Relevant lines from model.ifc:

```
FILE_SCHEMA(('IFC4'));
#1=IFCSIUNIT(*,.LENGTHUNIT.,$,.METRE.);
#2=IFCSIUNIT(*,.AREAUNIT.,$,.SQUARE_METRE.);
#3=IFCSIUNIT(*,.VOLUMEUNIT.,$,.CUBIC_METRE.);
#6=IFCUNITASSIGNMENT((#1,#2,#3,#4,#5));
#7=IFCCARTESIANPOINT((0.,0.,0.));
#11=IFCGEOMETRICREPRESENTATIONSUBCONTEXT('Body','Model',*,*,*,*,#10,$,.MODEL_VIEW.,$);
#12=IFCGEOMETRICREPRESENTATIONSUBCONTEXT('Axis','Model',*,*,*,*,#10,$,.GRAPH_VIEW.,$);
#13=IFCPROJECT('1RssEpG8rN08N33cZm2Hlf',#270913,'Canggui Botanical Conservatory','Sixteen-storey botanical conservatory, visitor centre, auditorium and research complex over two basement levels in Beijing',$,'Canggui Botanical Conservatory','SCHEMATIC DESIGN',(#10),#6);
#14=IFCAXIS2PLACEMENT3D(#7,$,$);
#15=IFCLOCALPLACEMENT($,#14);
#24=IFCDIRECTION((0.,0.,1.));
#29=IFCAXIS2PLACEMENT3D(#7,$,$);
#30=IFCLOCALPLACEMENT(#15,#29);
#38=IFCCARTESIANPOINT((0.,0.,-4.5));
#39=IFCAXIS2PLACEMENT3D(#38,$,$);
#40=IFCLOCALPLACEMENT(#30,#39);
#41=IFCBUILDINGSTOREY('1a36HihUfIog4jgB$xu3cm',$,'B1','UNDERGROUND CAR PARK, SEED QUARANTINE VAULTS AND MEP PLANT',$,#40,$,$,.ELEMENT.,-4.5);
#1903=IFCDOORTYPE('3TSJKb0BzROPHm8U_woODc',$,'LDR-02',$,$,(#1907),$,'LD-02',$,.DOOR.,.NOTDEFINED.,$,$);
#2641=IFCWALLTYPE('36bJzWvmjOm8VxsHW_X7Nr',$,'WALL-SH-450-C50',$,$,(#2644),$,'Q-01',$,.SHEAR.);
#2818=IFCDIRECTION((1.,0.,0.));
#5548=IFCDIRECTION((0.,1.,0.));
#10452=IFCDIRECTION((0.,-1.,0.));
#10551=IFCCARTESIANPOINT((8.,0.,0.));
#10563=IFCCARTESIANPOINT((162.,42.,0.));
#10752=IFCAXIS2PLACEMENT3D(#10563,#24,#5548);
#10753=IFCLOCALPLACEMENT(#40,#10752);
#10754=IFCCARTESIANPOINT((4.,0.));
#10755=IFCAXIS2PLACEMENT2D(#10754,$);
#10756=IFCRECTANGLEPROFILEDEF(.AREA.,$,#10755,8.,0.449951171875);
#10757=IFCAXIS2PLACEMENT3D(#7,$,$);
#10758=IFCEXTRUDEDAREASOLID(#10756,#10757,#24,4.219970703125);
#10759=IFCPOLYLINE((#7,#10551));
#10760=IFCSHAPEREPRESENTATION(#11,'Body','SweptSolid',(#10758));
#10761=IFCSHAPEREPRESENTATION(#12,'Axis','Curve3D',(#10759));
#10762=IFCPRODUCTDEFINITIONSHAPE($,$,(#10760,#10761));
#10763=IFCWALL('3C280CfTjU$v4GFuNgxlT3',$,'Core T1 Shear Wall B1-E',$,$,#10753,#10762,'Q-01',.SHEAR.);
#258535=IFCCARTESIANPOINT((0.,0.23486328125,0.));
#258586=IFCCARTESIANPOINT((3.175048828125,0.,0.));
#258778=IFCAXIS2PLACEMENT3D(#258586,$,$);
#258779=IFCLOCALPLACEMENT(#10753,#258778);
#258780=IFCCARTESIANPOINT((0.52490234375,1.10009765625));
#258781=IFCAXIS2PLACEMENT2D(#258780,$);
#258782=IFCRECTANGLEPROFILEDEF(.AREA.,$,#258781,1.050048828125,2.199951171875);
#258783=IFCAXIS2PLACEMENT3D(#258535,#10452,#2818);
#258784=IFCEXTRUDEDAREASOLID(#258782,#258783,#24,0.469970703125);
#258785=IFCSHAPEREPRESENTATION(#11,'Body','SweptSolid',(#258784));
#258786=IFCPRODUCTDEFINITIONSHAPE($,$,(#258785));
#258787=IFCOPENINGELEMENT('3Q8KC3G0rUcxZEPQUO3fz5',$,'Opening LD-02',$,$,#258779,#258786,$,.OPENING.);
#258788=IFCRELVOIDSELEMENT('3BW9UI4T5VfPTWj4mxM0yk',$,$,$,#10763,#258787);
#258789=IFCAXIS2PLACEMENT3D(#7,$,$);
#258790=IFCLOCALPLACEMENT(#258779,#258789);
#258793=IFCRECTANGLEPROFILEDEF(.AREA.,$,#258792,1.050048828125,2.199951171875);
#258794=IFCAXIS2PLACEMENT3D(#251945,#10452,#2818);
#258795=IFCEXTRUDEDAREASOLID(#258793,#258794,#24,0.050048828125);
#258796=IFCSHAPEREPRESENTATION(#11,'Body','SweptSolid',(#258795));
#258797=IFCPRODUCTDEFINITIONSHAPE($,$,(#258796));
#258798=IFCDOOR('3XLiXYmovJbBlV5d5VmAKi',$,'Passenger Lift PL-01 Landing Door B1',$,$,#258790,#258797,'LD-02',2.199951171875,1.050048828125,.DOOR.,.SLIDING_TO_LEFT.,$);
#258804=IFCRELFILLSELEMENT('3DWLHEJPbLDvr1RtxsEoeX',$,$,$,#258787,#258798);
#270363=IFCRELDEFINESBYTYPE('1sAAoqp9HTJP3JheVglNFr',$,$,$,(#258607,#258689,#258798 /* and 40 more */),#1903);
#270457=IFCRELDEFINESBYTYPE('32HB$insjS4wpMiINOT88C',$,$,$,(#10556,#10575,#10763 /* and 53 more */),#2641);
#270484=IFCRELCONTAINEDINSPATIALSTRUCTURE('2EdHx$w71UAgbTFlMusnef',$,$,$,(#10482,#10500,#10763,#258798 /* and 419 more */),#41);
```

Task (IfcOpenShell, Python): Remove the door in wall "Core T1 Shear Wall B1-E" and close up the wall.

```python
import ifcopenshell
import ifcopenshell.api.feature
import ifcopenshell.api.root
import ifcopenshell.geom
import ifcopenshell.util.shape

model = ifcopenshell.open("model.ifc")
settings = ifcopenshell.geom.settings()


def volume(element):
    """Net volume in cubic metres, openings subtracted."""
    shape = ifcopenshell.geom.create_shape(settings, element)
    return ifcopenshell.util.shape.get_volume(shape.geometry)


door = model.by_guid("3XLiXYmovJbBlV5d5VmAKi")
opening = door.FillsVoids[0].RelatingOpeningElement
wall = opening.VoidsElements[0].RelatingBuildingElement
before = volume(wall)

ifcopenshell.api.root.remove_product(model, product=door)
ifcopenshell.api.feature.remove_feature(model, feature=opening)

after = volume(wall)

print(f"wall volume {before:.3f} -> {after:.3f} m3")

model.write("model_rev.ifc")
```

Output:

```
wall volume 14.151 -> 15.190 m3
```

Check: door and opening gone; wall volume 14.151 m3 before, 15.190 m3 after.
